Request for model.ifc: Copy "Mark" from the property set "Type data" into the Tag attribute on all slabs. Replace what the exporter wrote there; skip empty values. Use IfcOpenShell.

First a look at what the model holds.

```python
import ifcopenshell
import ifcopenshell.util.element

model = ifcopenshell.open("model.ifc")
print(model.schema)
slabs = model.by_type("IfcSlab")
print(len(slabs), "slabs")
for e in slabs[:8]:
    source = ifcopenshell.util.element.get_pset(e, "Type data", "Mark")
    target = e.Tag
    print(e.id(), repr(source), repr(target), sep=" | ")
```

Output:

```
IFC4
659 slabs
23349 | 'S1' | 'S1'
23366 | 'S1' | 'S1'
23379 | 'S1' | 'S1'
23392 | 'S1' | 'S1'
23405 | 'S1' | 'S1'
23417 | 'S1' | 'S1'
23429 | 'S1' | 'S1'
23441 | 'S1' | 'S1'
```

```python
import ifcopenshell
import ifcopenshell.util.element

model = ifcopenshell.open("model.ifc")

count = 0
for e in model.by_type("IfcSlab"):
    value = ifcopenshell.util.element.get_pset(e, "Type data", "Mark")
    current = e.Tag
    if not value or not value.strip() or current == value:
        continue
    e.Tag = value
    count += 1

print(count, "slabs updated")

model.write("model_updated.ifc")
```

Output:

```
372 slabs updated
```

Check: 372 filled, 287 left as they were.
